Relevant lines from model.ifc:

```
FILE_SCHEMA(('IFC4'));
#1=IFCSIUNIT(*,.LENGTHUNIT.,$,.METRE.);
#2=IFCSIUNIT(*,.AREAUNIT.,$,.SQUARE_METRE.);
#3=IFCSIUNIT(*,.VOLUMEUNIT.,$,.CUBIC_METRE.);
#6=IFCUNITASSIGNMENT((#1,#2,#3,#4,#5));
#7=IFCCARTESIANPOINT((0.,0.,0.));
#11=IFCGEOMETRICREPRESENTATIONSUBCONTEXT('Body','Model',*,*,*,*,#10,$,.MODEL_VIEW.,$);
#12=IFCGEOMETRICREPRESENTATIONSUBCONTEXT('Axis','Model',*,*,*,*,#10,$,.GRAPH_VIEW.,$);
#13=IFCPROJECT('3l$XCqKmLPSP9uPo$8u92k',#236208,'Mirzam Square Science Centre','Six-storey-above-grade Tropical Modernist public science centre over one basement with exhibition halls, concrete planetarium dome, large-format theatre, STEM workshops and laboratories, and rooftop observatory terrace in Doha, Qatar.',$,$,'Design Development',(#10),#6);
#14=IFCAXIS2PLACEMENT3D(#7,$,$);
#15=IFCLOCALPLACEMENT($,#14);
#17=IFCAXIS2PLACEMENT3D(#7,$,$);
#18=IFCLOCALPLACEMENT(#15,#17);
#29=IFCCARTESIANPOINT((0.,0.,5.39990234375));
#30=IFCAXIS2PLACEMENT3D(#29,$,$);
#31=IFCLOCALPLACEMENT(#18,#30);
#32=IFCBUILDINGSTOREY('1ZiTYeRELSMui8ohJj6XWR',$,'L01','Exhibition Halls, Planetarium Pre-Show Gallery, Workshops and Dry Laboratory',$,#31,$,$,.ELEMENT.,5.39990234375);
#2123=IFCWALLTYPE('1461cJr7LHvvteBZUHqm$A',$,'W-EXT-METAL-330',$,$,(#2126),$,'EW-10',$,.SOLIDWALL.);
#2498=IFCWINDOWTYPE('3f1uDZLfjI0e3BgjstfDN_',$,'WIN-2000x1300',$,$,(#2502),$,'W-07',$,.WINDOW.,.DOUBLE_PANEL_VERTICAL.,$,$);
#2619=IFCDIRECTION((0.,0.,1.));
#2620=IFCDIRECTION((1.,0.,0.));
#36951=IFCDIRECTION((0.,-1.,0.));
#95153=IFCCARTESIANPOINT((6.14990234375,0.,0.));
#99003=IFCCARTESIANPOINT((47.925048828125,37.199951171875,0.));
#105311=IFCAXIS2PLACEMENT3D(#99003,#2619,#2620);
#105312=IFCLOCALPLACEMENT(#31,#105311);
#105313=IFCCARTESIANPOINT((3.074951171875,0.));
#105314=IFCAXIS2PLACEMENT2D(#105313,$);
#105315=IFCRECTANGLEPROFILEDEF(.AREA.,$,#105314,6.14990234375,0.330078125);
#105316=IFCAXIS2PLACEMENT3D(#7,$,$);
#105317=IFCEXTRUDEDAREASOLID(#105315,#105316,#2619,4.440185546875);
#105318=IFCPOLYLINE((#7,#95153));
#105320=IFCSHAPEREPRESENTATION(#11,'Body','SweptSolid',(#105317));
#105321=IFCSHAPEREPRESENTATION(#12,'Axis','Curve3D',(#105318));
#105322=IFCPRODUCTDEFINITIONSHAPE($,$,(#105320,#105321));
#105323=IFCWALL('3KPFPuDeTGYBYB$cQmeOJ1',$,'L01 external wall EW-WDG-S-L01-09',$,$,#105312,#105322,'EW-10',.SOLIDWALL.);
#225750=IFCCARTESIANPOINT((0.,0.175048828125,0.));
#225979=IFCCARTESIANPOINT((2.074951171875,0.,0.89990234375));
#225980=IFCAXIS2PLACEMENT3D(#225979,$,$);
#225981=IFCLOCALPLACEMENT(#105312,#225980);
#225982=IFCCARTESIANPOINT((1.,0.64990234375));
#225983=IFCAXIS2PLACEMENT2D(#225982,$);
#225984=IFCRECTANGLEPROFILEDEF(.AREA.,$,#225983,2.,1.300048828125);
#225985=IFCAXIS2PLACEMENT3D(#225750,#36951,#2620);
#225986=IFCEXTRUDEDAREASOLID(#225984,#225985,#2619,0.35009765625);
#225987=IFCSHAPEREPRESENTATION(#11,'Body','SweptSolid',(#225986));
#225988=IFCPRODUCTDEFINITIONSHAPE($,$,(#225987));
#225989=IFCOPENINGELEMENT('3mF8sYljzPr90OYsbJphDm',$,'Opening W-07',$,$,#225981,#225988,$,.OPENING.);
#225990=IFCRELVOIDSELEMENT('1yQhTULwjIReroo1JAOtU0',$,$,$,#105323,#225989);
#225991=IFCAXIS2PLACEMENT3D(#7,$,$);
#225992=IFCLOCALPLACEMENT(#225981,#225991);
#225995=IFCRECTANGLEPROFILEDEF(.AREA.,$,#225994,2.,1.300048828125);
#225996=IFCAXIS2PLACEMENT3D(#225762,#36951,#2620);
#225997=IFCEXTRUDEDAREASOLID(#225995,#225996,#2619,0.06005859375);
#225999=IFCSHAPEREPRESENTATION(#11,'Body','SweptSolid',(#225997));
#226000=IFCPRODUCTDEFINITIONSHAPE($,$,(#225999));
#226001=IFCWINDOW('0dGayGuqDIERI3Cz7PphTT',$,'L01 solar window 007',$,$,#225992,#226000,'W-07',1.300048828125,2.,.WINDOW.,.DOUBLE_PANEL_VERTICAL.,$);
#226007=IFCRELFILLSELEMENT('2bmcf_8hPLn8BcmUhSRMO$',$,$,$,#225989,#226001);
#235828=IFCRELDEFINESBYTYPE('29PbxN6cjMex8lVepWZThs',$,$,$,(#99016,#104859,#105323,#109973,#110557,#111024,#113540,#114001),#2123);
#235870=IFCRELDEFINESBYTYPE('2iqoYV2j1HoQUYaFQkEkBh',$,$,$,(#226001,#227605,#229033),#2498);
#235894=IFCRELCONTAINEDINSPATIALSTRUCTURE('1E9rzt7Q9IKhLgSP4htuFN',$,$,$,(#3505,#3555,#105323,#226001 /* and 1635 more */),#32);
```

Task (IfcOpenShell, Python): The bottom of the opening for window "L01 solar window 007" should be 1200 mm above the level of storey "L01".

```python
import numpy as np
import ifcopenshell
import ifcopenshell.api.geometry
import ifcopenshell.geom
import ifcopenshell.util.element
import ifcopenshell.util.placement
import ifcopenshell.util.shape
import ifcopenshell.util.unit

model = ifcopenshell.open("model.ifc")
unit_scale = ifcopenshell.util.unit.calculate_unit_scale(model)

window = model.by_guid("0dGayGuqDIERI3Cz7PphTT")
opening = window.FillsVoids[0].RelatingOpeningElement
storey = ifcopenshell.util.element.get_container(window, ifc_class="IfcBuildingStorey")
level = ifcopenshell.util.placement.get_local_placement(storey.ObjectPlacement)[2, 3]

# The opening's origin need not be at the sill, so measure its lowest point.
shape = ifcopenshell.geom.create_shape(ifcopenshell.geom.settings(), opening)
bottom = ifcopenshell.util.shape.get_shape_bottom_elevation(shape, shape.geometry) / unit_scale
dz = level + 1.2 / unit_scale - bottom

shift = np.array([0.0, 0.0, dz])
# The window is placed relative to its opening, so it follows when the opening moves.
matrix = ifcopenshell.util.placement.get_local_placement(opening.ObjectPlacement)
matrix[:3, 3] += shift
ifcopenshell.api.geometry.edit_object_placement(
    model, product=opening, matrix=matrix, is_si=False, should_transform_children=True
)

print(f"moved by {dz * unit_scale:+.3f} m")

model.write("model_v2.ifc")
```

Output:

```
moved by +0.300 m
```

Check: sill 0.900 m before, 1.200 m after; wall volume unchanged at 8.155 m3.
